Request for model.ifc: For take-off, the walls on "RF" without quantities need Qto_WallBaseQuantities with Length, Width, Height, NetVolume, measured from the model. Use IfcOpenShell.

First a look at what the model holds.

```python
import ifcopenshell
import ifcopenshell.util.element
import ifcopenshell.util.unit

model = ifcopenshell.open("model.ifc")
print(model.schema)
for unit_type in ("LENGTHUNIT", "AREAUNIT", "VOLUMEUNIT"):
    print(unit_type, ifcopenshell.util.unit.calculate_unit_scale(model, unit_type))
storey = next(s for s in model.by_type("IfcBuildingStorey") if s.Name == "RF")
walls = [e for e in ifcopenshell.util.element.get_decomposition(storey) if e.is_a("IfcWall")]
for e in sorted(walls, key=lambda e: e.id()):
    print(e.id(), e.is_a(), e.Name, list(ifcopenshell.util.element.get_psets(e, qtos_only=True)), sep=" | ")
```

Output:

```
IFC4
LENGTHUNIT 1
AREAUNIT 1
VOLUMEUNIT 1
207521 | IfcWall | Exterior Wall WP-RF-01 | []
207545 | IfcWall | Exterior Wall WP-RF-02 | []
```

```python
import ifcopenshell
import ifcopenshell.api.pset
import ifcopenshell.geom
import ifcopenshell.util.element
import ifcopenshell.util.shape
import ifcopenshell.util.unit

model = ifcopenshell.open("model.ifc")
unit_scale = ifcopenshell.util.unit.calculate_unit_scale(model)
volume_scale = ifcopenshell.util.unit.calculate_unit_scale(model, "VOLUMEUNIT")
settings = ifcopenshell.geom.settings()

storey = next(s for s in model.by_type("IfcBuildingStorey") if s.Name == "RF")
walls = [e for e in ifcopenshell.util.element.get_decomposition(storey) if e.is_a("IfcWall")]

for e in sorted(walls, key=lambda e: e.id()):
    if ifcopenshell.util.element.get_psets(e, qtos_only=True, should_inherit=False):
        continue
    # Geometry comes back in metres, in the element's own axes.
    shape = ifcopenshell.geom.create_shape(settings, e)
    values = {
        "Length": ifcopenshell.util.shape.get_x(shape.geometry) / unit_scale,
        "Width": ifcopenshell.util.shape.get_y(shape.geometry) / unit_scale,
        "Height": ifcopenshell.util.shape.get_z(shape.geometry) / unit_scale,
        "NetVolume": ifcopenshell.util.shape.get_volume(shape.geometry) / volume_scale,
    }
    qto = ifcopenshell.api.pset.add_qto(model, product=e, name="Qto_WallBaseQuantities")
    ifcopenshell.api.pset.edit_qto(model, qto=qto, properties=values)
    print(e.id(), {k: round(v, 3) for k, v in values.items()})

model.write("model_edited.ifc")
```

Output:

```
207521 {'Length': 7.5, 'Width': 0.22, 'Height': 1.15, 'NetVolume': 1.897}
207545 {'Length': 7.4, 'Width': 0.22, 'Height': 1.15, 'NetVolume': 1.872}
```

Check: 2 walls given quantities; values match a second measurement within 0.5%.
